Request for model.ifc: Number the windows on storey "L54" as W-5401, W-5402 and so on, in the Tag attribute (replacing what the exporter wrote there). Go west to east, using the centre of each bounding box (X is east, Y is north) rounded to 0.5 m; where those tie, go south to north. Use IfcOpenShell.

First a look at what the model holds.

```python
import ifcopenshell
import ifcopenshell.util.element
import ifcopenshell.util.placement

model = ifcopenshell.open("model.ifc")
print(model.schema)
storey = next(s for s in model.by_type("IfcBuildingStorey") if s.Name == "L54")
windows = [e for e in ifcopenshell.util.element.get_decomposition(storey) if e.is_a("IfcWindow")]
for e in sorted(windows, key=lambda e: e.id()):
    origin = ifcopenshell.util.placement.get_local_placement(e.ObjectPlacement)[:3, 3]
    print(e.id(), e.Tag, e.Name, origin.round(2) + 0.0, sep=" | ")
```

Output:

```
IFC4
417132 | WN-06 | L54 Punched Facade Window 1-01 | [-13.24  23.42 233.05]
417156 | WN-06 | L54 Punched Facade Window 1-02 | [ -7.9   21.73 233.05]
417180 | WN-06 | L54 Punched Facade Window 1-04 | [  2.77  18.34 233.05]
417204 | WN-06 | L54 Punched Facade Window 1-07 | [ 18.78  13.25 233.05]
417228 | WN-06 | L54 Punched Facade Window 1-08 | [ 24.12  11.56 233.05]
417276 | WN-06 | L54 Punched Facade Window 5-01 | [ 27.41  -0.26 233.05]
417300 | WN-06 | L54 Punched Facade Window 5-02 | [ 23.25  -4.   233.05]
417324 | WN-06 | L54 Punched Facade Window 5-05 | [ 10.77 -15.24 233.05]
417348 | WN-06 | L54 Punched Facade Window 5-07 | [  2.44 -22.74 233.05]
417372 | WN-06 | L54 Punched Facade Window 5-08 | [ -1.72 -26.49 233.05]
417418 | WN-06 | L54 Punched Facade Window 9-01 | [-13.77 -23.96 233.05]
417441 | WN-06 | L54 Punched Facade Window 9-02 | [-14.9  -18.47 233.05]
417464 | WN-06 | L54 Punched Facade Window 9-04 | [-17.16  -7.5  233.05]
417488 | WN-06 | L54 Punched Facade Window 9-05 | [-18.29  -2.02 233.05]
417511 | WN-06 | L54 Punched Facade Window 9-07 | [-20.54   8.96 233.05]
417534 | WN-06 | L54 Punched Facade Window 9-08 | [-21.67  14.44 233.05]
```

```python
import ifcopenshell
import ifcopenshell.geom
import ifcopenshell.util.element
import ifcopenshell.util.shape

model = ifcopenshell.open("model.ifc")
settings = ifcopenshell.geom.settings()
settings.set("use-world-coords", True)


def centre(element):
    shape = ifcopenshell.geom.create_shape(settings, element)
    return ifcopenshell.util.shape.get_bbox_centroid(shape.geometry)


storey = next(s for s in model.by_type("IfcBuildingStorey") if s.Name == "L54")
windows = [e for e in ifcopenshell.util.element.get_decomposition(storey) if e.is_a("IfcWindow")]

# Insertion points can sit at a corner or the storey origin, so sort by the geometry (in metres).
centres = {e: centre(e) for e in windows}
windows.sort(key=lambda e: (round(centres[e][0] / 0.5), centres[e][1]))

for i, e in enumerate(windows, start=1):
    number = f"W-54{i:02d}"
    e.Tag = number
    print(e.id(), number)

model.write("model-out.ifc")
```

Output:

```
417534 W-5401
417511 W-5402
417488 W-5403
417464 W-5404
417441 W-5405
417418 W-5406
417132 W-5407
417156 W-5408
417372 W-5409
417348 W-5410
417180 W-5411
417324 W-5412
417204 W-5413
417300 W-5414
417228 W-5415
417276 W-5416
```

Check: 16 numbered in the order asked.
